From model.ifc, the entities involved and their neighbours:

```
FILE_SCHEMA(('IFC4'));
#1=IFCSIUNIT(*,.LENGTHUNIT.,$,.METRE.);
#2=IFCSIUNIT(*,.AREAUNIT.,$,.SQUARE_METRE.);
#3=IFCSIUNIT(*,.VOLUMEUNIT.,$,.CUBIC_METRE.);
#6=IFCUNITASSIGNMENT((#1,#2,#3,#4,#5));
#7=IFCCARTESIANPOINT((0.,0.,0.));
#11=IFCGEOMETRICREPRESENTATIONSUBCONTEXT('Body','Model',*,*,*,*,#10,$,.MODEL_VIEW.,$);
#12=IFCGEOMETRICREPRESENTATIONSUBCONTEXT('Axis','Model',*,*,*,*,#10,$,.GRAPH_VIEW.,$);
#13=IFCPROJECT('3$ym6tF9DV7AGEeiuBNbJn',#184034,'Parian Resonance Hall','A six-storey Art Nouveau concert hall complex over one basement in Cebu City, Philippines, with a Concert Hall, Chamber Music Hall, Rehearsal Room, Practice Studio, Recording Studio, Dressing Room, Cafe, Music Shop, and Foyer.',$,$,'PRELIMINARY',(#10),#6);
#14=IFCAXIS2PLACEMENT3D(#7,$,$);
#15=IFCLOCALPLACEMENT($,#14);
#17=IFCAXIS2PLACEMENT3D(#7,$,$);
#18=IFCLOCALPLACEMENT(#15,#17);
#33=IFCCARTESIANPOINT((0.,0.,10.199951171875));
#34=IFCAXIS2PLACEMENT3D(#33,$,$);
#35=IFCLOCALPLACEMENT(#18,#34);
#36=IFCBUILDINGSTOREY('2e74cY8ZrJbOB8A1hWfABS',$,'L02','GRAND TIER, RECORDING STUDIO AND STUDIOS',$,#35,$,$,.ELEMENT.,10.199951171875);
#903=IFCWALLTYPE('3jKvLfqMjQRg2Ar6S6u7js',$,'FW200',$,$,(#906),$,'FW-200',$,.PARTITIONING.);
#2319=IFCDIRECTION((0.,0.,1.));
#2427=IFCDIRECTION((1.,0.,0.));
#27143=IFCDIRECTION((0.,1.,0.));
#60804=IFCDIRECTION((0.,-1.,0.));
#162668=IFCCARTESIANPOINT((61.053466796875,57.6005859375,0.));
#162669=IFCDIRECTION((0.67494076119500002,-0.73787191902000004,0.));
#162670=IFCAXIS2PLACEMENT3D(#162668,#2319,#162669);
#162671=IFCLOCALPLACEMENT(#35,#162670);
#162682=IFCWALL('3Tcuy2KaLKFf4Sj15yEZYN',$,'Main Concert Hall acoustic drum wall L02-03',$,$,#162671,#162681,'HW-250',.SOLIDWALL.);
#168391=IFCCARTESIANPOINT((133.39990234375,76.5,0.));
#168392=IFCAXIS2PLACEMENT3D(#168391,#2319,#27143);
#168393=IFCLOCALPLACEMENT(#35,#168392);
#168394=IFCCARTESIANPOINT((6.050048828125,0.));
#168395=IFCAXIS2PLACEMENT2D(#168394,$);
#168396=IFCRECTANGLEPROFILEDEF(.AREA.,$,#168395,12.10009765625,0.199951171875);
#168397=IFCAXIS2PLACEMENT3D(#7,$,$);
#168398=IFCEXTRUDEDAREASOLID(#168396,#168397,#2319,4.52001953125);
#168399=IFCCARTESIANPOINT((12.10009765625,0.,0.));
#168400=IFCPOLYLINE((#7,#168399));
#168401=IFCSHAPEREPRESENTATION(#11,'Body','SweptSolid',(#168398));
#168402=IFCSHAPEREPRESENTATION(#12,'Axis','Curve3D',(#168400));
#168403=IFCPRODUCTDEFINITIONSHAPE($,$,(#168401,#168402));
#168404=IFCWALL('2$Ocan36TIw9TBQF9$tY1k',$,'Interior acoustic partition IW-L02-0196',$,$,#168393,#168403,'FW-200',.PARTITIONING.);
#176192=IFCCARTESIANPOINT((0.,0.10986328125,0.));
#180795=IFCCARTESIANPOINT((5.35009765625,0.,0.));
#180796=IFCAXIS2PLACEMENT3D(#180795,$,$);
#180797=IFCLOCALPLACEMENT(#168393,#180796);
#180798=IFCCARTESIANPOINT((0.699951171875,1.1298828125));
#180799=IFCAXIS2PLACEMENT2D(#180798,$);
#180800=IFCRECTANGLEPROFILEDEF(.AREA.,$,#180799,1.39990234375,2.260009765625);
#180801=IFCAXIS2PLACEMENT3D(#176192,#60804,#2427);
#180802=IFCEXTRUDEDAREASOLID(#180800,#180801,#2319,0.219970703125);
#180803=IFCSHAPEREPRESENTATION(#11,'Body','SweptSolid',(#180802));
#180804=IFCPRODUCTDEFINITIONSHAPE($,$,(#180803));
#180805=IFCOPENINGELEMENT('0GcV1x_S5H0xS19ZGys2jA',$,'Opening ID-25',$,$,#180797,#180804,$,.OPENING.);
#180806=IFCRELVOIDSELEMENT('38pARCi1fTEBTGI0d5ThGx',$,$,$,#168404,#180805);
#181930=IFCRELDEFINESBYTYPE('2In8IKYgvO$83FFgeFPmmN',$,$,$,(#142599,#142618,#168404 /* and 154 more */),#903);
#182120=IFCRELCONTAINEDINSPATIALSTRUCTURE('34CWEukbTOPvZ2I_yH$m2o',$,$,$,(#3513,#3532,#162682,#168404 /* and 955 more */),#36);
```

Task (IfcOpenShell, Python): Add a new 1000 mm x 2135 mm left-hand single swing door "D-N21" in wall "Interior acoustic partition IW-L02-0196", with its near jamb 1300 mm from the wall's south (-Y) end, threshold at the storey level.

```python
import numpy as np
import ifcopenshell
import ifcopenshell.api.feature
import ifcopenshell.api.geometry
import ifcopenshell.api.root
import ifcopenshell.api.spatial
import ifcopenshell.geom
import ifcopenshell.util.element
import ifcopenshell.util.placement
import ifcopenshell.util.representation
import ifcopenshell.util.shape
import ifcopenshell.util.unit

model = ifcopenshell.open("model.ifc")
unit_scale = ifcopenshell.util.unit.calculate_unit_scale(model)
settings = ifcopenshell.geom.settings()


def volume(element):
    """Net volume in cubic metres, openings subtracted."""
    shape = ifcopenshell.geom.create_shape(settings, element)
    return ifcopenshell.util.shape.get_volume(shape.geometry)


wall = model.by_guid("2$Ocan36TIw9TBQF9$tY1k")
storey = ifcopenshell.util.element.get_container(wall, ifc_class="IfcBuildingStorey")
context = ifcopenshell.util.representation.get_context(model, "Model", "Body", "MODEL_VIEW")
before = volume(wall)

width, height, from_end, sill = 1, 2.135, 1.3, 0.0  # metres

# The wall runs along its own X axis, and the end named is its -X end.
wall_shape = ifcopenshell.geom.create_shape(settings, wall)
x, y, z = ifcopenshell.util.shape.get_vertices(wall_shape.geometry).T
start = x.min() + from_end
face, thickness = float(y.min()), float(y.max() - y.min())
wall_matrix = ifcopenshell.util.placement.get_local_placement(wall.ObjectPlacement)
level = ifcopenshell.util.placement.get_local_placement(storey.ObjectPlacement)[2, 3]


def in_wall(x, y):
    """Placement at x, y metres in the wall's axes, at sill height."""
    matrix = wall_matrix.copy()
    matrix[:, 3] = wall_matrix @ np.array([x / unit_scale, y / unit_scale, 0.0, 1.0])
    matrix[2, 3] = level + sill / unit_scale
    return matrix


# Opening: a box that overshoots both wall faces by 50 mm.
opening = ifcopenshell.api.root.create_entity(model, ifc_class="IfcOpeningElement", predefined_type="OPENING")
box = ifcopenshell.api.geometry.add_wall_representation(
    model, context=context, length=width, height=height, thickness=thickness + 0.1
)
ifcopenshell.api.geometry.assign_representation(model, product=opening, representation=box)
ifcopenshell.api.geometry.edit_object_placement(model, product=opening, matrix=in_wall(start, face - 0.05), is_si=False)
ifcopenshell.api.feature.add_feature(model, feature=opening, element=wall)

door = ifcopenshell.api.root.create_entity(model, ifc_class="IfcDoor", name="D-N21", predefined_type="DOOR")
door.OverallWidth, door.OverallHeight = width / unit_scale, height / unit_scale
door.OperationType = "SINGLE_SWING_LEFT"
body = ifcopenshell.api.geometry.add_door_representation(
    model,
    context=context,
    overall_width=door.OverallWidth,
    overall_height=door.OverallHeight,
    operation_type="SINGLE_SWING_LEFT",
    lining_properties={"LiningDepth": thickness / unit_scale, "ThresholdDepth": thickness / unit_scale},
)
ifcopenshell.api.geometry.assign_representation(model, product=door, representation=body)
ifcopenshell.api.spatial.assign_container(model, products=[door], relating_structure=storey)
ifcopenshell.api.feature.add_filling(model, opening=opening, element=door)

# The lining spans the wall, so the door starts at the wall face.
ifcopenshell.api.geometry.edit_object_placement(model, product=door, matrix=in_wall(start, face), is_si=False)

after = volume(wall)

print(f"wall volume {before:.3f} -> {after:.3f} m3")

model.write("model_v2.ifc")
```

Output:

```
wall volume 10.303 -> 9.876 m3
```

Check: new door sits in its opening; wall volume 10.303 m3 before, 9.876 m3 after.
